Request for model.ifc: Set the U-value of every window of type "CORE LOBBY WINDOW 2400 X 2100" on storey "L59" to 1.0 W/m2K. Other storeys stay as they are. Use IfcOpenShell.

First a look at what the model holds.

```python
import ifcopenshell
import ifcopenshell.util.element

model = ifcopenshell.open("model.ifc")
print(model.schema)
storey = next(s for s in model.by_type("IfcBuildingStorey") if s.Name == "L59")
windows = [e for e in ifcopenshell.util.element.get_decomposition(storey) if e.is_a("IfcWindow")]
seen = {}
for e in windows:
    element_type = ifcopenshell.util.element.get_type(e)
    key = (element_type.Name if element_type != e and element_type else None, ifcopenshell.util.element.get_pset(e, "Pset_WindowCommon", "ThermalTransmittance"))
    seen[key] = seen.get(key, 0) + 1
for (name, value), count in sorted(seen.items(), key=str):
    print(count, "x", name, "|", value)
```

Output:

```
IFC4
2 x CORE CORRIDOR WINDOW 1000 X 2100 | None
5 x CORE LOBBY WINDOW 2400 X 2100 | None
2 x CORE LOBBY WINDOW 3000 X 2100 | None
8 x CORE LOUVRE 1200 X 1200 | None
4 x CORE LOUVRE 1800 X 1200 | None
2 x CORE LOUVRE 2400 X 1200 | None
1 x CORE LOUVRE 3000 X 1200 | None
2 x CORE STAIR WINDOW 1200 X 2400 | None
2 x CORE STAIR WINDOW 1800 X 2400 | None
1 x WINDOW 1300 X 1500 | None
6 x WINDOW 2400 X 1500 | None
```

```python
import ifcopenshell
import ifcopenshell.api.pset
import ifcopenshell.util.element

model = ifcopenshell.open("model.ifc")

storey = next(s for s in model.by_type("IfcBuildingStorey") if s.Name == "L59")
windows = [e for e in ifcopenshell.util.element.get_decomposition(storey) if e.is_a("IfcWindow")]

count = 0
for e in windows:
    element_type = ifcopenshell.util.element.get_type(e)
    if element_type in (None, e) or element_type.Name != "CORE LOBBY WINDOW 2400 X 2100":
        continue
    found = ifcopenshell.util.element.get_pset(e, "Pset_WindowCommon", should_inherit=False)
    if found:
        pset = model.by_id(found["id"])
        if len(ifcopenshell.util.element.get_elements_by_pset(pset)) > 1:
            pset = ifcopenshell.api.pset.unshare_pset(model, products=[e], pset=pset)[0]
    else:
        pset = ifcopenshell.api.pset.add_pset(model, product=e, name="Pset_WindowCommon")
    ifcopenshell.api.pset.edit_pset(model, pset=pset, properties={"ThermalTransmittance": 1.0})
    count += 1

print(count, "windows updated")

model.write("model_edited.ifc")
```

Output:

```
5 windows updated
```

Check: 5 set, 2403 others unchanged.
